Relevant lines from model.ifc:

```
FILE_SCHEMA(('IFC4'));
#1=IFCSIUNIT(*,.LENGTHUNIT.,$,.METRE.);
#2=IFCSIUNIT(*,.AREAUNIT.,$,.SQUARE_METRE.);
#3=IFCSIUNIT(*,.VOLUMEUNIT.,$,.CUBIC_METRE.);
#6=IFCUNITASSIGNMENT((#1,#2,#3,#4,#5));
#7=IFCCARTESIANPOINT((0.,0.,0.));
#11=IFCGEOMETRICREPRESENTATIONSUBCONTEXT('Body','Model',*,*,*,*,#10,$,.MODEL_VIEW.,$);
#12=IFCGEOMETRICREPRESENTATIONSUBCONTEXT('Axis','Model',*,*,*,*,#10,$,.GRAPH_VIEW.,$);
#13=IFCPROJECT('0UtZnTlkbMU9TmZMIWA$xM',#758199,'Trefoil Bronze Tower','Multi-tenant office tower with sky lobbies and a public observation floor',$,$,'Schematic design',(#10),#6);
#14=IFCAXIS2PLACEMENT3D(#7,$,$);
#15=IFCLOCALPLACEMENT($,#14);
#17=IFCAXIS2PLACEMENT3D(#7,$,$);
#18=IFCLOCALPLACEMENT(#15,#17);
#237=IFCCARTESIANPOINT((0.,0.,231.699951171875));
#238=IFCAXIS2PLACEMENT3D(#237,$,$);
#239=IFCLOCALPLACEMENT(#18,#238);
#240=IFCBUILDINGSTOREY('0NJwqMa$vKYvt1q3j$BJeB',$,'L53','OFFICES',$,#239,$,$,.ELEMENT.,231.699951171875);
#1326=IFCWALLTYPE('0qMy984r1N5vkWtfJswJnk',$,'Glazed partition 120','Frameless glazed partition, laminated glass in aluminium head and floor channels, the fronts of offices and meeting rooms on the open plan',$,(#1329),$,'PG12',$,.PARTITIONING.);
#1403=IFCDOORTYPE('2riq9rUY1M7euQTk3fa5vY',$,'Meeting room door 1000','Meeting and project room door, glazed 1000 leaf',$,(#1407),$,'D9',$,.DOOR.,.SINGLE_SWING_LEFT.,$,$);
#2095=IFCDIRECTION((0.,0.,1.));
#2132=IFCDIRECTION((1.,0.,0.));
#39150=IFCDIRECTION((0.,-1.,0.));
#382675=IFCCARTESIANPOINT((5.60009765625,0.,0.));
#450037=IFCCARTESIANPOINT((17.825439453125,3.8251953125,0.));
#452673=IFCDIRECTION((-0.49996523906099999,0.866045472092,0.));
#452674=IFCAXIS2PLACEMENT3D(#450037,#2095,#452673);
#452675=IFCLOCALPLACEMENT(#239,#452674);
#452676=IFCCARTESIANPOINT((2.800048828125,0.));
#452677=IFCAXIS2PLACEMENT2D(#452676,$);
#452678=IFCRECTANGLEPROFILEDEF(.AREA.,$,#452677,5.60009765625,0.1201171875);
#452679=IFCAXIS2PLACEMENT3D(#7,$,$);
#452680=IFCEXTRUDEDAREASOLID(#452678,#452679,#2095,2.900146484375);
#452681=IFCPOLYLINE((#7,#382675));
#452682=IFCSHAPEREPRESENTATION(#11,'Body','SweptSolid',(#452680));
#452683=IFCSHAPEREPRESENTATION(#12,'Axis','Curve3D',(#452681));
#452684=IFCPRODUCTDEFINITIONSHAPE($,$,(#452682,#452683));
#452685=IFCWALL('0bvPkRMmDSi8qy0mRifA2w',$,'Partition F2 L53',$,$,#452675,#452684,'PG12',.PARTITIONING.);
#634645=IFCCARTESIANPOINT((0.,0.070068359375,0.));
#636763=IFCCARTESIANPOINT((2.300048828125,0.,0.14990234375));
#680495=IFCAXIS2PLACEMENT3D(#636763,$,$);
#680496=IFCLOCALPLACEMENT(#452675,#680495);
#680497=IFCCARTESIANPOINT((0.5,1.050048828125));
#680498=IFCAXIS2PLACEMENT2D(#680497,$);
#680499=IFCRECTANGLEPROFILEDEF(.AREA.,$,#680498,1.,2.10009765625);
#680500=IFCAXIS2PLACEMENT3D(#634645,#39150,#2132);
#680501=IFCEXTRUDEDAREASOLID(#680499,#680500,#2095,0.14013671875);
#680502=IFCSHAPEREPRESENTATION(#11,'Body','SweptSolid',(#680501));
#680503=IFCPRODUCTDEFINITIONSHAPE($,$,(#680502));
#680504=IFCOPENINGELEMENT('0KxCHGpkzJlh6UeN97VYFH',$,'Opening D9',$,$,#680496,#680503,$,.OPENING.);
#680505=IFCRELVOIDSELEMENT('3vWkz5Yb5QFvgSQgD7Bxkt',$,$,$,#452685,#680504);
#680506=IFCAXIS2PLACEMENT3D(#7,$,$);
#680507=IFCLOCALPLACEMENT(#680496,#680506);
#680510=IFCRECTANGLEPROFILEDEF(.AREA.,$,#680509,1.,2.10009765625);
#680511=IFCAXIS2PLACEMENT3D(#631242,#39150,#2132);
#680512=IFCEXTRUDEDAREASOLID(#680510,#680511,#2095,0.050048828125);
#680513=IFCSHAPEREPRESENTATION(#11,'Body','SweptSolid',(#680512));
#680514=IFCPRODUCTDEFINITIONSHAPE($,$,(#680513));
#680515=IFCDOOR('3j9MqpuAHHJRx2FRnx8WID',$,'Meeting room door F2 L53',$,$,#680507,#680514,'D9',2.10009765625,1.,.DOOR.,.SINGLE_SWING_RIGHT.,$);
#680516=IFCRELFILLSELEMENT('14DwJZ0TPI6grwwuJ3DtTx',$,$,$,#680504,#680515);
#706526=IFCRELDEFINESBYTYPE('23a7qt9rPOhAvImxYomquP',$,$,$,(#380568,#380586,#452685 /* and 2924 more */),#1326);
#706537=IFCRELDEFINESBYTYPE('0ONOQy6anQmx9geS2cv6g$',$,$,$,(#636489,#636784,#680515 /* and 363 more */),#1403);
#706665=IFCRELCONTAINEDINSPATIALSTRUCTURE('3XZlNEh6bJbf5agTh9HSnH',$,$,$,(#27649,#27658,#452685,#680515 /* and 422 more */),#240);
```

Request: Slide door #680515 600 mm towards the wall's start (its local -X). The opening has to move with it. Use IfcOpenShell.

```python
import ifcopenshell
import ifcopenshell.api.geometry
import ifcopenshell.util.placement
import ifcopenshell.util.unit

model = ifcopenshell.open("model.ifc")
unit_scale = ifcopenshell.util.unit.calculate_unit_scale(model)

door = model.by_guid("3j9MqpuAHHJRx2FRnx8WID")
opening = door.FillsVoids[0].RelatingOpeningElement
wall = opening.VoidsElements[0].RelatingBuildingElement

wall_matrix = ifcopenshell.util.placement.get_local_placement(wall.ObjectPlacement)
shift = wall_matrix[:3, 0] * -0.6 / unit_scale
before = ifcopenshell.util.placement.get_local_placement(door.ObjectPlacement)[:3, 3].copy()

# The door is placed relative to its opening, so it follows when the opening moves.
matrix = ifcopenshell.util.placement.get_local_placement(opening.ObjectPlacement)
matrix[:3, 3] += shift
ifcopenshell.api.geometry.edit_object_placement(
    model, product=opening, matrix=matrix, is_si=False, should_transform_children=True
)

after = ifcopenshell.util.placement.get_local_placement(door.ObjectPlacement)[:3, 3]
print("door moved by", (after - before).round(3) + 0.0)

model.write("model_edited.ifc")
```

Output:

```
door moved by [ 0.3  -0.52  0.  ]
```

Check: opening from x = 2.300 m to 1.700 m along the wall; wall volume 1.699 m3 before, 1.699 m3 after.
